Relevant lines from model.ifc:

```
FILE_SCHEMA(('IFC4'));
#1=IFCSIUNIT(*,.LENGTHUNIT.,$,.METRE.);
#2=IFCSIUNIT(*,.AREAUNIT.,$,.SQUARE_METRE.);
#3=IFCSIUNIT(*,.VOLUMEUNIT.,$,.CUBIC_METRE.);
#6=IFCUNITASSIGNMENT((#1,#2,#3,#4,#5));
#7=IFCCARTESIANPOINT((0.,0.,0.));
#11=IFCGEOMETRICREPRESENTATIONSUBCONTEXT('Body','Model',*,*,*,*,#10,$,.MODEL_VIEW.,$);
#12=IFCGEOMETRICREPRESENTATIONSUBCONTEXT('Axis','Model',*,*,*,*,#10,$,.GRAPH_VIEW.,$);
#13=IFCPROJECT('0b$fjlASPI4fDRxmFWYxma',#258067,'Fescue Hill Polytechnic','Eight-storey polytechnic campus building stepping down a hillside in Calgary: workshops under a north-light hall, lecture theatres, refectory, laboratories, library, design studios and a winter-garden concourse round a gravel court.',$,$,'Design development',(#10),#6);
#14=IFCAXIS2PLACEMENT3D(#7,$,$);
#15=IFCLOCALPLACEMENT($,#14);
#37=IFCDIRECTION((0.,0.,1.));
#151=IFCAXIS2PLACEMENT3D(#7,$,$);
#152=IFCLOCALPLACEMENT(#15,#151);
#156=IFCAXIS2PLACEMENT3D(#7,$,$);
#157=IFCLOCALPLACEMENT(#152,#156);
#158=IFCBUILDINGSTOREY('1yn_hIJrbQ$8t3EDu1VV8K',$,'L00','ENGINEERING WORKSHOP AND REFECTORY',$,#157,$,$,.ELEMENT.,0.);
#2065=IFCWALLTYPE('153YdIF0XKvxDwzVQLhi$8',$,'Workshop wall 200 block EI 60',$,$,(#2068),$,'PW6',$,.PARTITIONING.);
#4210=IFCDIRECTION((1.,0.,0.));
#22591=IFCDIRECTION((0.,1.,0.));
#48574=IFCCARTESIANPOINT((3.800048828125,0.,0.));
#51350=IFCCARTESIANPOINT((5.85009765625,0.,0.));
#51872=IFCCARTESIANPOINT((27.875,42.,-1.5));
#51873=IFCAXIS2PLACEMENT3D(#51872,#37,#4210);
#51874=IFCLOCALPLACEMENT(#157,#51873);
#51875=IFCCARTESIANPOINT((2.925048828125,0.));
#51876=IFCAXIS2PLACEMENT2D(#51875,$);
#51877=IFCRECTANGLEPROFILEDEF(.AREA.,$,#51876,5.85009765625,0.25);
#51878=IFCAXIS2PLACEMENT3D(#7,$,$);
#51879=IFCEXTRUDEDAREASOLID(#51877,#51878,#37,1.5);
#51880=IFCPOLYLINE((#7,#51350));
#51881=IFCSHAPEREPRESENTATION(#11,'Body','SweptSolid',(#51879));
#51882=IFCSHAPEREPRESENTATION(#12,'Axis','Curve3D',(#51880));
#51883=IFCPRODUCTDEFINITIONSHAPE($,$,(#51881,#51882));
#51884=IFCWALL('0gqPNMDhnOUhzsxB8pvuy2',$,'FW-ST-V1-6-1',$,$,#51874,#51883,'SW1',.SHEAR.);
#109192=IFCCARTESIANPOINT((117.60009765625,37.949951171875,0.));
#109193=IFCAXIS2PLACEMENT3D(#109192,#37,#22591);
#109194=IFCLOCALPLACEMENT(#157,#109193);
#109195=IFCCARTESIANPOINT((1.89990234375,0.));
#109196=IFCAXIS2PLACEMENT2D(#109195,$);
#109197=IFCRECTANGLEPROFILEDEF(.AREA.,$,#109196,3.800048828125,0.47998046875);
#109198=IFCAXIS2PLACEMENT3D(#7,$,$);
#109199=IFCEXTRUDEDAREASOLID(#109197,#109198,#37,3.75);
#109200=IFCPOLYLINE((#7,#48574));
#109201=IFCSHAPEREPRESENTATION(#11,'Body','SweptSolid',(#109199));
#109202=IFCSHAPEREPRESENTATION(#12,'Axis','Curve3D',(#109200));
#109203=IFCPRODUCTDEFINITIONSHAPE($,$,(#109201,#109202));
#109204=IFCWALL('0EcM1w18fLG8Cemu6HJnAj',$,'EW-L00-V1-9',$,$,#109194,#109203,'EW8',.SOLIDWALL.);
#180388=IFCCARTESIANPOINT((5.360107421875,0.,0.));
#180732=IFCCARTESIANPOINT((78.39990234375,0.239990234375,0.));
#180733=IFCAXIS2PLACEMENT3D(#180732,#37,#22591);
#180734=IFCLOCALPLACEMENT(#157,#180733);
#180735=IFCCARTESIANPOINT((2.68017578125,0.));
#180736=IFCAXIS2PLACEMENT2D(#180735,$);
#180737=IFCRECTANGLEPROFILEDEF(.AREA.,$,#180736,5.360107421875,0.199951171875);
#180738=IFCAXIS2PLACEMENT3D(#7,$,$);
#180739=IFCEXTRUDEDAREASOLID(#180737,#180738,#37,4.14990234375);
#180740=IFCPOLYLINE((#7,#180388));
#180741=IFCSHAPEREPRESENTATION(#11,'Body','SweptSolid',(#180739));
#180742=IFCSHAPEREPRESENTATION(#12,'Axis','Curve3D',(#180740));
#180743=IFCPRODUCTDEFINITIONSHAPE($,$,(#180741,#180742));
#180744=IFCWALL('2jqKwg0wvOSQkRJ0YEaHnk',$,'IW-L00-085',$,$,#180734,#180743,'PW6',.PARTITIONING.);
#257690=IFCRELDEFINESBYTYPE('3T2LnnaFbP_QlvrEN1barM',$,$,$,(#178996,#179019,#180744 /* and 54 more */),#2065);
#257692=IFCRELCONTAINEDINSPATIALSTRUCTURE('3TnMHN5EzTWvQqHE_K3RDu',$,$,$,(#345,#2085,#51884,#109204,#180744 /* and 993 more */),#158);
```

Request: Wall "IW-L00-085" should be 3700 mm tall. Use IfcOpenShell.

```python
import ifcopenshell
import ifcopenshell.geom
import ifcopenshell.util.representation
import ifcopenshell.util.shape
import ifcopenshell.util.unit

model = ifcopenshell.open("model.ifc")
unit_scale = ifcopenshell.util.unit.calculate_unit_scale(model)
settings = ifcopenshell.geom.settings()


def volume(element):
    """Net volume in cubic metres, openings subtracted."""
    shape = ifcopenshell.geom.create_shape(settings, element)
    return ifcopenshell.util.shape.get_volume(shape.geometry)


wall = model.by_id(180744)
before = volume(wall)

body = ifcopenshell.util.representation.get_representation(wall, "Model", "Body")
solid = body.Items[0]
old_height = solid.Depth
solid.Depth = 3.7 / unit_scale
after = volume(wall)

print(f"height {old_height:g} -> {solid.Depth:g}, volume {before:.3f} -> {after:.3f} m3")

model.write("model-out.ifc")
```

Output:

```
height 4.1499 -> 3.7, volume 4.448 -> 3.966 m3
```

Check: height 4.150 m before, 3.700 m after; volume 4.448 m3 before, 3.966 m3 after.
